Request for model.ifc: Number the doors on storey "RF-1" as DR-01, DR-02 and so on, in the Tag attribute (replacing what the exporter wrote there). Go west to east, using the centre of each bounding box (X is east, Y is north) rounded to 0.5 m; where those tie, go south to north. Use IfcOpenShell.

First a look at what the model holds.

```python
import ifcopenshell
import ifcopenshell.util.element
import ifcopenshell.util.placement

model = ifcopenshell.open("model.ifc")
print(model.schema)
storey = next(s for s in model.by_type("IfcBuildingStorey") if s.Name == "RF-1")
doors = [e for e in ifcopenshell.util.element.get_decomposition(storey) if e.is_a("IfcDoor")]
for e in sorted(doors, key=lambda e: e.id()):
    origin = ifcopenshell.util.placement.get_local_placement(e.ObjectPlacement)[:3, 3]
    print(e.id(), e.Tag, e.Name, origin.round(2) + 0.0, sep=" | ")
```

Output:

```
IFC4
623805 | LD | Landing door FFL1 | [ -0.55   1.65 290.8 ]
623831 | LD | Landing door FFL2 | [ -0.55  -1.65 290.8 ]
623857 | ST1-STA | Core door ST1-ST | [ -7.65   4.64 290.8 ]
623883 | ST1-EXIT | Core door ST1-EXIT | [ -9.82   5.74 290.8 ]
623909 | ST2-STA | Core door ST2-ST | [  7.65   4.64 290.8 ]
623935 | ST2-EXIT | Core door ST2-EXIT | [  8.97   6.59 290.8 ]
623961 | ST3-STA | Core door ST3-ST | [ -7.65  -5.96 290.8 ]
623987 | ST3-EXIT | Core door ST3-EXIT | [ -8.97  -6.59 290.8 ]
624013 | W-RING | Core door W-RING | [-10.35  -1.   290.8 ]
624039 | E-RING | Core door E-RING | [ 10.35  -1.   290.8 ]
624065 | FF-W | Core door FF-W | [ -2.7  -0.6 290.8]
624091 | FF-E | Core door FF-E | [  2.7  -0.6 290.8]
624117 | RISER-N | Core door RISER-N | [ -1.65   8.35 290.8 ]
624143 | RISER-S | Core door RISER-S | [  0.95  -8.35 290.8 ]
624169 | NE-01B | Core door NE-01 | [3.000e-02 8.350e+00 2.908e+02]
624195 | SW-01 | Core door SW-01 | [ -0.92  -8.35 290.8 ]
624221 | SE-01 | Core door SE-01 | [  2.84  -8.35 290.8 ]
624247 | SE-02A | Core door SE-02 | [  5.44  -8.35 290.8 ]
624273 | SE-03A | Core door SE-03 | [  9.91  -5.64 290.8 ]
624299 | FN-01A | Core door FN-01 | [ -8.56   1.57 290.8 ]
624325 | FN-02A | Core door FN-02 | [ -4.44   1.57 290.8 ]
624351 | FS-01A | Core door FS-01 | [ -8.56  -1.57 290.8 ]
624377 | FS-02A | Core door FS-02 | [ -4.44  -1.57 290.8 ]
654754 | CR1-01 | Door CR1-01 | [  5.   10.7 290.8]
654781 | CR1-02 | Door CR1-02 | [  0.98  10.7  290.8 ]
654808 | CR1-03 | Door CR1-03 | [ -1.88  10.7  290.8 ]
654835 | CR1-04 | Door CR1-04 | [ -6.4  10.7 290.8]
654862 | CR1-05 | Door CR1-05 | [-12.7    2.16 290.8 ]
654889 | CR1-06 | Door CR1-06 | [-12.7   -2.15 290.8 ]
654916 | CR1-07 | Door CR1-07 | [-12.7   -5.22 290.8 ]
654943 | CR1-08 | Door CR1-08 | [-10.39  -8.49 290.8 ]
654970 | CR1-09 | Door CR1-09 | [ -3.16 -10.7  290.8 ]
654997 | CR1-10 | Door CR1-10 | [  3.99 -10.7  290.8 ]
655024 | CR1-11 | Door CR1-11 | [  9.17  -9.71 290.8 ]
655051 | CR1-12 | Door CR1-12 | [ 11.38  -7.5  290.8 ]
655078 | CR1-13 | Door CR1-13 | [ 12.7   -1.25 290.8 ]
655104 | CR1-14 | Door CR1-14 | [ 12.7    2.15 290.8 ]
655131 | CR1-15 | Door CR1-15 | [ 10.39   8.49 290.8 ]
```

```python
import ifcopenshell
import ifcopenshell.geom
import ifcopenshell.util.element
import ifcopenshell.util.shape

model = ifcopenshell.open("model.ifc")
settings = ifcopenshell.geom.settings()
settings.set("use-world-coords", True)


def centre(element):
    shape = ifcopenshell.geom.create_shape(settings, element)
    return ifcopenshell.util.shape.get_bbox_centroid(shape.geometry)


storey = next(s for s in model.by_type("IfcBuildingStorey") if s.Name == "RF-1")
doors = [e for e in ifcopenshell.util.element.get_decomposition(storey) if e.is_a("IfcDoor")]

# Insertion points can sit at a corner or the storey origin, so sort by the geometry (in metres).
centres = {e: centre(e) for e in doors}
doors.sort(key=lambda e: (round(centres[e][0] / 0.5), centres[e][1]))

for i, e in enumerate(doors, start=1):
    number = f"DR-{i:02d}"
    e.Tag = number
    print(e.id(), number)

model.write("model_updated.ifc")
```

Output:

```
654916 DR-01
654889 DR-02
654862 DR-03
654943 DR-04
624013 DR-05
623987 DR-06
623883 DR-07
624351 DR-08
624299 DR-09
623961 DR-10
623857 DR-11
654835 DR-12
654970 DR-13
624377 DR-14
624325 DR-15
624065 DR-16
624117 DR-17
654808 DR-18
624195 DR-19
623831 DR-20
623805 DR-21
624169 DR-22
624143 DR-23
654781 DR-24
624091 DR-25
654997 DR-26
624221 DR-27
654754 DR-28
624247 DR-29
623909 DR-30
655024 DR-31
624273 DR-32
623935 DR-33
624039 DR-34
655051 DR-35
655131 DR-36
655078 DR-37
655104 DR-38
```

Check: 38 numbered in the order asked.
